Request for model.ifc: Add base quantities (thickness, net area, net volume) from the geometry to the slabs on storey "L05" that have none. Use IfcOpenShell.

First a look at what the model holds.

```python
import ifcopenshell
import ifcopenshell.util.element
import ifcopenshell.util.unit

model = ifcopenshell.open("model.ifc")
print(model.schema)
for unit_type in ("LENGTHUNIT", "AREAUNIT", "VOLUMEUNIT"):
    print(unit_type, ifcopenshell.util.unit.calculate_unit_scale(model, unit_type))
storey = next(s for s in model.by_type("IfcBuildingStorey") if s.Name == "L05")
slabs = [e for e in ifcopenshell.util.element.get_decomposition(storey) if e.is_a("IfcSlab")]
for e in sorted(slabs, key=lambda e: e.id()):
    print(e.id(), e.is_a(), e.Name, list(ifcopenshell.util.element.get_psets(e, qtos_only=True)), sep=" | ")
```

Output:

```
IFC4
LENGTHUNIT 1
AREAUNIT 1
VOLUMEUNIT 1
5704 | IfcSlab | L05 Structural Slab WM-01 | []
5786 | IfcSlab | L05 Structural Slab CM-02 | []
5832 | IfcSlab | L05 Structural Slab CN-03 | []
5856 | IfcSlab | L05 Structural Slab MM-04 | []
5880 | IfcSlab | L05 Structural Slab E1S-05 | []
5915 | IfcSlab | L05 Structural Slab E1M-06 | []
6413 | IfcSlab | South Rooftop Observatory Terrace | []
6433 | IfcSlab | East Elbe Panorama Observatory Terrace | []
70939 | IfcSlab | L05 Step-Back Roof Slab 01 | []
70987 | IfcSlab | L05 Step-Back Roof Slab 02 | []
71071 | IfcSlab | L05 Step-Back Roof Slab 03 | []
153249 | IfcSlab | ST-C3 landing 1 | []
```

```python
import ifcopenshell
import ifcopenshell.api.pset
import ifcopenshell.geom
import ifcopenshell.util.element
import ifcopenshell.util.shape
import ifcopenshell.util.unit

model = ifcopenshell.open("model.ifc")
unit_scale = ifcopenshell.util.unit.calculate_unit_scale(model)
area_scale = ifcopenshell.util.unit.calculate_unit_scale(model, "AREAUNIT")
volume_scale = ifcopenshell.util.unit.calculate_unit_scale(model, "VOLUMEUNIT")
settings = ifcopenshell.geom.settings()

storey = next(s for s in model.by_type("IfcBuildingStorey") if s.Name == "L05")
slabs = [e for e in ifcopenshell.util.element.get_decomposition(storey) if e.is_a("IfcSlab")]

for e in sorted(slabs, key=lambda e: e.id()):
    if ifcopenshell.util.element.get_psets(e, qtos_only=True, should_inherit=False):
        continue
    # Geometry comes back in metres, in the element's own axes.
    shape = ifcopenshell.geom.create_shape(settings, e)
    values = {
        "Width": ifcopenshell.util.shape.get_z(shape.geometry) / unit_scale,
        "NetArea": ifcopenshell.util.shape.get_footprint_area(shape.geometry) / area_scale,
        "NetVolume": ifcopenshell.util.shape.get_volume(shape.geometry) / volume_scale,
    }
    qto = ifcopenshell.api.pset.add_qto(model, product=e, name="Qto_SlabBaseQuantities")
    ifcopenshell.api.pset.edit_qto(model, qto=qto, properties=values)
    print(e.id(), {k: round(v, 3) for k, v in values.items()})

model.write("model_updated.ifc")
```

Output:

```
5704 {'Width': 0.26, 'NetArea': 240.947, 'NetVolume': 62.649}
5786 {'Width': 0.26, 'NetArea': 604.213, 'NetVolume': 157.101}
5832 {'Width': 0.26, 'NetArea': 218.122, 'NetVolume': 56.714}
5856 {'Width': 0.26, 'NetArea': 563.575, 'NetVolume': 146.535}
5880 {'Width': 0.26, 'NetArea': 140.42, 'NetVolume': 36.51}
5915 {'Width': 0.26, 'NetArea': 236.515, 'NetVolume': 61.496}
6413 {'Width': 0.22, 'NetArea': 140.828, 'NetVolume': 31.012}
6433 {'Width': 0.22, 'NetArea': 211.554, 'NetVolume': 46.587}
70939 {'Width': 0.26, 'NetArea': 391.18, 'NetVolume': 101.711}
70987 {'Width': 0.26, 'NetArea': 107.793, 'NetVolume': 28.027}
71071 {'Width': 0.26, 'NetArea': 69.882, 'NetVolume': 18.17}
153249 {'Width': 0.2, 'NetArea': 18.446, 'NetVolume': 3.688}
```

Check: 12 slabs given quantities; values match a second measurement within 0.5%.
